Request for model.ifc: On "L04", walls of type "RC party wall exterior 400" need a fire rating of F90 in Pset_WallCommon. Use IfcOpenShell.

First a look at what the model holds.

```python
import ifcopenshell
import ifcopenshell.util.element

model = ifcopenshell.open("model.ifc")
print(model.schema)
storey = next(s for s in model.by_type("IfcBuildingStorey") if s.Name == "L04")
walls = [e for e in ifcopenshell.util.element.get_decomposition(storey) if e.is_a("IfcWall")]
seen = {}
for e in walls:
    element_type = ifcopenshell.util.element.get_type(e)
    key = (element_type.Name if element_type != e and element_type else None, ifcopenshell.util.element.get_pset(e, "Pset_WallCommon", "FireRating"))
    seen[key] = seen.get(key, 0) + 1
for (name, value), count in sorted(seen.items(), key=str):
    print(count, "x", name, "|", value)
```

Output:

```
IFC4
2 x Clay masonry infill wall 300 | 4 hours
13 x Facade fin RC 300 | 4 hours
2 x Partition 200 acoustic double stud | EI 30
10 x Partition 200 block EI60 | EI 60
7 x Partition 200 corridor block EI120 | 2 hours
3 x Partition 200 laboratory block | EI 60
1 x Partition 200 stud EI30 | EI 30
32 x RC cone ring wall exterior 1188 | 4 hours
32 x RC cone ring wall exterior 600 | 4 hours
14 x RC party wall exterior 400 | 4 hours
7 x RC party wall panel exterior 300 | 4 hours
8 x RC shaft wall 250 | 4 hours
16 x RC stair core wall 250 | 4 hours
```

```python
import ifcopenshell
import ifcopenshell.api.pset
import ifcopenshell.util.element

model = ifcopenshell.open("model.ifc")

storey = next(s for s in model.by_type("IfcBuildingStorey") if s.Name == "L04")
walls = [e for e in ifcopenshell.util.element.get_decomposition(storey) if e.is_a("IfcWall")]

count = 0
for e in walls:
    element_type = ifcopenshell.util.element.get_type(e)
    if element_type in (None, e) or element_type.Name != "RC party wall exterior 400":
        continue
    # add_pset returns the element's existing set when there is one.
    pset = ifcopenshell.api.pset.add_pset(model, product=e, name="Pset_WallCommon")
    ifcopenshell.api.pset.edit_pset(model, pset=pset, properties={"FireRating": "F90"})
    count += 1

print(count, "walls updated")

model.write("model_edited.ifc")
```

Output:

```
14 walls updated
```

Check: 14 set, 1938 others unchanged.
